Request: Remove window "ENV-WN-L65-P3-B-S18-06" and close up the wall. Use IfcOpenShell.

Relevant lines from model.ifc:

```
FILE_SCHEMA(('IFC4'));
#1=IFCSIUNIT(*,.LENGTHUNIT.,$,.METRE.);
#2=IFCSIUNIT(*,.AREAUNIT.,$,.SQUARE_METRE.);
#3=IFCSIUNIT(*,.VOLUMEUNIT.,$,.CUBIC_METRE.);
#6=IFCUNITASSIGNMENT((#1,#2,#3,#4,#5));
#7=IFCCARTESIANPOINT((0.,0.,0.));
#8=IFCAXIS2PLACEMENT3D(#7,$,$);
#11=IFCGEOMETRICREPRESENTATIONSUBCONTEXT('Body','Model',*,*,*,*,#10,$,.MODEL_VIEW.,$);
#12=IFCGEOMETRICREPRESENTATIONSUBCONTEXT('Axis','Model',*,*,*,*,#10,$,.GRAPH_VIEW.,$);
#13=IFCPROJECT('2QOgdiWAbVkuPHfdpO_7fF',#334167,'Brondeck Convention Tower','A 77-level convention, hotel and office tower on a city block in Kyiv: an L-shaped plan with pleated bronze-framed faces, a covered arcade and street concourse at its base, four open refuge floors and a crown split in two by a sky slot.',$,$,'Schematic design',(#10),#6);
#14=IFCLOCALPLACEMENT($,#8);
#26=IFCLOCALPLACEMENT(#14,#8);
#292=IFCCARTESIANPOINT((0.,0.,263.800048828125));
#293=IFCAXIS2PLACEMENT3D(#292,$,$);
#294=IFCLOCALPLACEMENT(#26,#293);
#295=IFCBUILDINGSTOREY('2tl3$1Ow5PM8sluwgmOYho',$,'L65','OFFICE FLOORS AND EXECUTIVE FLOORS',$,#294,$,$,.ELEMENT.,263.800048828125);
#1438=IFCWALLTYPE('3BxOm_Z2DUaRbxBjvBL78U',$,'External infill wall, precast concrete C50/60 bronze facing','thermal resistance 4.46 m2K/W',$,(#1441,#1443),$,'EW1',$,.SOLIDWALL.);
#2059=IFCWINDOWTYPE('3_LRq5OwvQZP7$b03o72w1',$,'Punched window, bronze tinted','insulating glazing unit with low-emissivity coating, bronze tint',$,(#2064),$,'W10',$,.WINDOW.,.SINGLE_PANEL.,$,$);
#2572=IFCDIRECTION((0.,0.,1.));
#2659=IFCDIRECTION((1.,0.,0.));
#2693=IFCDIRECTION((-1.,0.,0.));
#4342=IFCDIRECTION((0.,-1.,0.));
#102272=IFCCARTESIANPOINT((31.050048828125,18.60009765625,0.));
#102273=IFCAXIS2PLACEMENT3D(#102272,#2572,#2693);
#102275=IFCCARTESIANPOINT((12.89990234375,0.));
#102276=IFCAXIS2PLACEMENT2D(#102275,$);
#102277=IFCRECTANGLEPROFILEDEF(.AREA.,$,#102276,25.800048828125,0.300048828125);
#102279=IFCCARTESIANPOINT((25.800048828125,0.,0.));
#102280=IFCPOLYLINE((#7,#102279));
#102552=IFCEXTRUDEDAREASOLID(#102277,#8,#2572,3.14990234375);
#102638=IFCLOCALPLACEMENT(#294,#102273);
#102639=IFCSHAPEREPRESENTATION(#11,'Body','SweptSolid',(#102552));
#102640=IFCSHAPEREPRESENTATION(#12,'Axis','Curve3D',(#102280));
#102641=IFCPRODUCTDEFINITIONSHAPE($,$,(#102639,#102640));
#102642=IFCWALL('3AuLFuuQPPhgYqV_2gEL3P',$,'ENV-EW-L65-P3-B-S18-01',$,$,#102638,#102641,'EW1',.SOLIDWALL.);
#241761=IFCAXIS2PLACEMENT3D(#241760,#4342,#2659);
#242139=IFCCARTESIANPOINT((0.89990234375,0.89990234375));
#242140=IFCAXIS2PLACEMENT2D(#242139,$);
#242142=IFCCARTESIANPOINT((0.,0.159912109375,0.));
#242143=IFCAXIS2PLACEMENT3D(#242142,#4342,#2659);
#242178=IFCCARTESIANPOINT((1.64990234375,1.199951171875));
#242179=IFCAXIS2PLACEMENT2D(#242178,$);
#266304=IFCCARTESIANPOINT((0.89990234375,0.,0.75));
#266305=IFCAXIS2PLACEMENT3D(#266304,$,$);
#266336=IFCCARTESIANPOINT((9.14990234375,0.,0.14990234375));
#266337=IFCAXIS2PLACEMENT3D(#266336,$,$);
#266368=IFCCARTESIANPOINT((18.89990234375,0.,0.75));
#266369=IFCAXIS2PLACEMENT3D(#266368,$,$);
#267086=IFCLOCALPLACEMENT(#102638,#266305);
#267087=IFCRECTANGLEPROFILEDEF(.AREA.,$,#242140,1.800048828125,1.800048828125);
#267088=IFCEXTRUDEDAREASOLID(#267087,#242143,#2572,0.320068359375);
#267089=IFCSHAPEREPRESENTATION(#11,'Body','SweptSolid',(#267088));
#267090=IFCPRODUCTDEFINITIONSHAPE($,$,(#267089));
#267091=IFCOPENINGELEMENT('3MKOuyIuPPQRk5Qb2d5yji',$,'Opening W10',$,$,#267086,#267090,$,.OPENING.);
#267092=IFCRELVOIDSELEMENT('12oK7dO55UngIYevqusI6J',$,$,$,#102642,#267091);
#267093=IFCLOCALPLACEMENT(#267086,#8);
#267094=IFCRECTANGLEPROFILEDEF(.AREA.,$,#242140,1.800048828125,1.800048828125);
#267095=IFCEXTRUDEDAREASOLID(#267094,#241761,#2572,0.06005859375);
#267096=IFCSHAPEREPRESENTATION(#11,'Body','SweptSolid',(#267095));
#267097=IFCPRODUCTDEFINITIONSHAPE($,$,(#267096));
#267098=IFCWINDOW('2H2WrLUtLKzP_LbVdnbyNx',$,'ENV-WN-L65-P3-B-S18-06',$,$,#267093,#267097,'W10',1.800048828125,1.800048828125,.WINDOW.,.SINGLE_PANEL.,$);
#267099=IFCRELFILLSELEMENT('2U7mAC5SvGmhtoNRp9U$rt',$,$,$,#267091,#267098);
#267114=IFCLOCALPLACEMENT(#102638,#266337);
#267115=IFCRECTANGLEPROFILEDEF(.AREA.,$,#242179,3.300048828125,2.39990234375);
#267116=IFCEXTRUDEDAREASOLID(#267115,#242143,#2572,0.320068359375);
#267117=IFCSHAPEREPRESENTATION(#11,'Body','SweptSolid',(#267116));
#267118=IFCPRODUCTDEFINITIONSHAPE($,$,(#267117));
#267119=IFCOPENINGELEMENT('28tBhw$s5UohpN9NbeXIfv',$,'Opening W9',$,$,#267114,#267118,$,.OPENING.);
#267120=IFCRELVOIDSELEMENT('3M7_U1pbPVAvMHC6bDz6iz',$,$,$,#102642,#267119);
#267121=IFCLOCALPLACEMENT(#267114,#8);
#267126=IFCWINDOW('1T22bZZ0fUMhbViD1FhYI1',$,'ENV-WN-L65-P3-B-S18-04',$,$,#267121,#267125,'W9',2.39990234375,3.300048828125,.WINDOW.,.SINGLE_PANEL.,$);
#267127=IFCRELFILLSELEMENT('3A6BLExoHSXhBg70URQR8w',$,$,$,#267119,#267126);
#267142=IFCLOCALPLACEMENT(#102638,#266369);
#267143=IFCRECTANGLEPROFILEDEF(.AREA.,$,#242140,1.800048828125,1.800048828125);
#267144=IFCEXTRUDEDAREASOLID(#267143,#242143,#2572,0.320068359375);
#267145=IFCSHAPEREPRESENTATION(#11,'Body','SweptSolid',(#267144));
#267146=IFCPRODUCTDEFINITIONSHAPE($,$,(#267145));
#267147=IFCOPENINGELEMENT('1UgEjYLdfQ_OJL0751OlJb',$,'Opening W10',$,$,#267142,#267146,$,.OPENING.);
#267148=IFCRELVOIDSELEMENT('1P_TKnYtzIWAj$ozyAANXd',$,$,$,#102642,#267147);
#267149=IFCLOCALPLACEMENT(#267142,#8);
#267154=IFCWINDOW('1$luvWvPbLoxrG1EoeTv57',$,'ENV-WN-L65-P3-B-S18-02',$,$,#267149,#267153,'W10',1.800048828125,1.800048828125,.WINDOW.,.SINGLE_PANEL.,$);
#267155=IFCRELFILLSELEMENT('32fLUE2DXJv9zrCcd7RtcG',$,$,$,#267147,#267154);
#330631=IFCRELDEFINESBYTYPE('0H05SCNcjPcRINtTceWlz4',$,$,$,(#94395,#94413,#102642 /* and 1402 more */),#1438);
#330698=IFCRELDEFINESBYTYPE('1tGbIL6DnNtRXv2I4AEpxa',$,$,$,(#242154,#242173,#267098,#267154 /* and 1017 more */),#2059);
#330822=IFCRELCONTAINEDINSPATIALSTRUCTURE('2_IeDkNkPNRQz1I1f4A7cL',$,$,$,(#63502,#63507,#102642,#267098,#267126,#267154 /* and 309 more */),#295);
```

```python
import ifcopenshell
import ifcopenshell.api.feature
import ifcopenshell.api.root
import ifcopenshell.geom
import ifcopenshell.util.shape

model = ifcopenshell.open("model.ifc")
settings = ifcopenshell.geom.settings()


def volume(element):
    """Net volume in cubic metres, openings subtracted."""
    shape = ifcopenshell.geom.create_shape(settings, element)
    return ifcopenshell.util.shape.get_volume(shape.geometry)


window = model.by_guid("2H2WrLUtLKzP_LbVdnbyNx")
opening = window.FillsVoids[0].RelatingOpeningElement
wall = opening.VoidsElements[0].RelatingBuildingElement
before = volume(wall)

ifcopenshell.api.root.remove_product(model, product=window)
ifcopenshell.api.feature.remove_feature(model, feature=opening)

after = volume(wall)

print(f"wall volume {before:.3f} -> {after:.3f} m3")

model.write("model_edited.ifc")
```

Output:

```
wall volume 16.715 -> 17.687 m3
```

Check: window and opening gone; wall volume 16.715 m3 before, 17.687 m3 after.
